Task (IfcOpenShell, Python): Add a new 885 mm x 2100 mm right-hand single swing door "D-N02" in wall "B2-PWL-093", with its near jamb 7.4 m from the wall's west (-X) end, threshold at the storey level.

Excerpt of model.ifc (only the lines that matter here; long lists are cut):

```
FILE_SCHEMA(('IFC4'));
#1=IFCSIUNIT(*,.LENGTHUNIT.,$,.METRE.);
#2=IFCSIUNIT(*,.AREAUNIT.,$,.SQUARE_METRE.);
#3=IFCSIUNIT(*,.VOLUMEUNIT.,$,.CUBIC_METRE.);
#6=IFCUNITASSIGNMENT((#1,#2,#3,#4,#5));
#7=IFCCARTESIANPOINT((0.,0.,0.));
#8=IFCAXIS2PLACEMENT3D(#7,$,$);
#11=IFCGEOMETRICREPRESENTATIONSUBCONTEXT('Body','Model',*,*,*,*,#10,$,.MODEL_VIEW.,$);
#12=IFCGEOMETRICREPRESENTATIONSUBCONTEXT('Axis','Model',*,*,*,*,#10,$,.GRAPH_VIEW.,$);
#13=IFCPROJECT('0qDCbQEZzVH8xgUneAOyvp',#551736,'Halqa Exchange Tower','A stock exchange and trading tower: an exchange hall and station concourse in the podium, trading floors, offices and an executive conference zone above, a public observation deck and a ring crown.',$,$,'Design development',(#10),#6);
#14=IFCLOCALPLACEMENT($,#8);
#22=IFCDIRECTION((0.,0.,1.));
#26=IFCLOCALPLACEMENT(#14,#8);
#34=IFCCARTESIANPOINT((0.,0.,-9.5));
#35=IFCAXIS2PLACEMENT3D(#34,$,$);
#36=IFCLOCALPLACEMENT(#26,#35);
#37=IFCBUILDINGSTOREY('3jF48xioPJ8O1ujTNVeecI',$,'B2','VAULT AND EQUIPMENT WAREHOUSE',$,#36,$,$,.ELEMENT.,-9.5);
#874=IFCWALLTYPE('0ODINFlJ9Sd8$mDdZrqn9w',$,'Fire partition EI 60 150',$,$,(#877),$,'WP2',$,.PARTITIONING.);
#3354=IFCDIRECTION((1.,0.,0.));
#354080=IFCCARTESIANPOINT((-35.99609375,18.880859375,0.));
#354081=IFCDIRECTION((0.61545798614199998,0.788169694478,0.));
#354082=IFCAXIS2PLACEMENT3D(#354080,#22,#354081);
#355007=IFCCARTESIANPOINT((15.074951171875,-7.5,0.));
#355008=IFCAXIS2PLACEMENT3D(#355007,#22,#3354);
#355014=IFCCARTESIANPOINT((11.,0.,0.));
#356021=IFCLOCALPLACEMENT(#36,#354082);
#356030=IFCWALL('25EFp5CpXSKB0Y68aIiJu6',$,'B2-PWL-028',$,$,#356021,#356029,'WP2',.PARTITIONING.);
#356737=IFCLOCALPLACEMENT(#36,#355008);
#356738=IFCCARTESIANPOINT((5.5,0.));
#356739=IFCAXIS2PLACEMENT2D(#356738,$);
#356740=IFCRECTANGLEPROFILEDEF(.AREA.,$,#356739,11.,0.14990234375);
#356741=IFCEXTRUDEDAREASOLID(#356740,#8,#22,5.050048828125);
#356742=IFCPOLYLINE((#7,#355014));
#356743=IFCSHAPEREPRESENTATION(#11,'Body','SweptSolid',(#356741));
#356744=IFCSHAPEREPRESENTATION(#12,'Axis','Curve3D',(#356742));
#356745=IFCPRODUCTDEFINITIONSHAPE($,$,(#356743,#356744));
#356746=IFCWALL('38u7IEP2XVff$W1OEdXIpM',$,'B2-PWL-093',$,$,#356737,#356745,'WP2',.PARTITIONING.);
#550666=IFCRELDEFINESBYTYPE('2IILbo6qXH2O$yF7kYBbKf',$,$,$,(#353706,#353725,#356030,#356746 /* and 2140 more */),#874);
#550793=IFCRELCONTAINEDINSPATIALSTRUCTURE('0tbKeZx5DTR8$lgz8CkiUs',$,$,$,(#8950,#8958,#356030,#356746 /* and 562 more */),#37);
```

```python
import numpy as np
import ifcopenshell
import ifcopenshell.api.feature
import ifcopenshell.api.geometry
import ifcopenshell.api.root
import ifcopenshell.api.spatial
import ifcopenshell.geom
import ifcopenshell.util.element
import ifcopenshell.util.placement
import ifcopenshell.util.representation
import ifcopenshell.util.shape
import ifcopenshell.util.unit

model = ifcopenshell.open("model.ifc")
unit_scale = ifcopenshell.util.unit.calculate_unit_scale(model)
settings = ifcopenshell.geom.settings()


def volume(element):
    """Net volume in cubic metres, openings subtracted."""
    shape = ifcopenshell.geom.create_shape(settings, element)
    return ifcopenshell.util.shape.get_volume(shape.geometry)


wall = model.by_guid("38u7IEP2XVff$W1OEdXIpM")
storey = ifcopenshell.util.element.get_container(wall, ifc_class="IfcBuildingStorey")
context = ifcopenshell.util.representation.get_context(model, "Model", "Body", "MODEL_VIEW")
before = volume(wall)

width, height, from_end, sill = 0.885, 2.1, 7.4, 0.0  # metres

# The wall runs along its own X axis, and the end named is its -X end.
wall_shape = ifcopenshell.geom.create_shape(settings, wall)
x, y, z = ifcopenshell.util.shape.get_vertices(wall_shape.geometry).T
start = x.min() + from_end
face, thickness = float(y.min()), float(y.max() - y.min())
wall_matrix = ifcopenshell.util.placement.get_local_placement(wall.ObjectPlacement)
level = ifcopenshell.util.placement.get_local_placement(storey.ObjectPlacement)[2, 3]


def in_wall(x, y):
    """Placement at x, y metres in the wall's axes, at sill height."""
    matrix = wall_matrix.copy()
    matrix[:, 3] = wall_matrix @ np.array([x / unit_scale, y / unit_scale, 0.0, 1.0])
    matrix[2, 3] = level + sill / unit_scale
    return matrix


# Opening: a box that overshoots both wall faces by 50 mm.
opening = ifcopenshell.api.root.create_entity(model, ifc_class="IfcOpeningElement", predefined_type="OPENING")
box = ifcopenshell.api.geometry.add_wall_representation(
    model, context=context, length=width, height=height, thickness=thickness + 0.1
)
ifcopenshell.api.geometry.assign_representation(model, product=opening, representation=box)
ifcopenshell.api.geometry.edit_object_placement(model, product=opening, matrix=in_wall(start, face - 0.05), is_si=False)
ifcopenshell.api.feature.add_feature(model, feature=opening, element=wall)

door = ifcopenshell.api.root.create_entity(model, ifc_class="IfcDoor", name="D-N02", predefined_type="DOOR")
door.OverallWidth, door.OverallHeight = width / unit_scale, height / unit_scale
door.OperationType = "SINGLE_SWING_RIGHT"
body = ifcopenshell.api.geometry.add_door_representation(
    model,
    context=context,
    overall_width=door.OverallWidth,
    overall_height=door.OverallHeight,
    operation_type="SINGLE_SWING_RIGHT",
    lining_properties={"LiningDepth": thickness / unit_scale, "ThresholdDepth": thickness / unit_scale},
)
ifcopenshell.api.geometry.assign_representation(model, product=door, representation=body)
ifcopenshell.api.spatial.assign_container(model, products=[door], relating_structure=storey)
ifcopenshell.api.feature.add_filling(model, opening=opening, element=door)

# The lining spans the wall, so the door starts at the wall face.
ifcopenshell.api.geometry.edit_object_placement(model, product=door, matrix=in_wall(start, face), is_si=False)

after = volume(wall)

print(f"wall volume {before:.3f} -> {after:.3f} m3")

model.write("model-out.ifc")
```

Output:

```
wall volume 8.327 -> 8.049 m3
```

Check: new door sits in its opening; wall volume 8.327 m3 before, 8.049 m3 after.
